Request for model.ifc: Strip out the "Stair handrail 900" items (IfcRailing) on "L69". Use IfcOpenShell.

First a look at what the model holds.

```python
import ifcopenshell
import ifcopenshell.util.element

model = ifcopenshell.open("model.ifc")
print(model.schema)
storey = next(s for s in model.by_type("IfcBuildingStorey") if s.Name == "L69")
railings = [e for e in ifcopenshell.util.element.get_decomposition(storey) if e.is_a("IfcRailing")]
seen = {}
for e in railings:
    element_type = ifcopenshell.util.element.get_type(e)
    name = element_type.Name if element_type not in (None, e) else None
    seen[name] = seen.get(name, 0) + 1
for name, count in sorted(seen.items(), key=str):
    print(count, "x", name)
```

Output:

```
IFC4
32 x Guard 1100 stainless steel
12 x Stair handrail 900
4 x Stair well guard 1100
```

```python
import ifcopenshell
import ifcopenshell.api.root
import ifcopenshell.util.element

model = ifcopenshell.open("model.ifc")

storey = next(s for s in model.by_type("IfcBuildingStorey") if s.Name == "L69")
railings = [e for e in ifcopenshell.util.element.get_decomposition(storey) if e.is_a("IfcRailing")]
targets = [e for e in railings if (t := ifcopenshell.util.element.get_type(e)) not in (None, e) and t.Name == "Stair handrail 900"]

for e in targets:
    ifcopenshell.api.root.remove_product(model, product=e)
print(len(targets), "removed")

model.write("model_v2.ifc")
```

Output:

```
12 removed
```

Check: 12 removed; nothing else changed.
